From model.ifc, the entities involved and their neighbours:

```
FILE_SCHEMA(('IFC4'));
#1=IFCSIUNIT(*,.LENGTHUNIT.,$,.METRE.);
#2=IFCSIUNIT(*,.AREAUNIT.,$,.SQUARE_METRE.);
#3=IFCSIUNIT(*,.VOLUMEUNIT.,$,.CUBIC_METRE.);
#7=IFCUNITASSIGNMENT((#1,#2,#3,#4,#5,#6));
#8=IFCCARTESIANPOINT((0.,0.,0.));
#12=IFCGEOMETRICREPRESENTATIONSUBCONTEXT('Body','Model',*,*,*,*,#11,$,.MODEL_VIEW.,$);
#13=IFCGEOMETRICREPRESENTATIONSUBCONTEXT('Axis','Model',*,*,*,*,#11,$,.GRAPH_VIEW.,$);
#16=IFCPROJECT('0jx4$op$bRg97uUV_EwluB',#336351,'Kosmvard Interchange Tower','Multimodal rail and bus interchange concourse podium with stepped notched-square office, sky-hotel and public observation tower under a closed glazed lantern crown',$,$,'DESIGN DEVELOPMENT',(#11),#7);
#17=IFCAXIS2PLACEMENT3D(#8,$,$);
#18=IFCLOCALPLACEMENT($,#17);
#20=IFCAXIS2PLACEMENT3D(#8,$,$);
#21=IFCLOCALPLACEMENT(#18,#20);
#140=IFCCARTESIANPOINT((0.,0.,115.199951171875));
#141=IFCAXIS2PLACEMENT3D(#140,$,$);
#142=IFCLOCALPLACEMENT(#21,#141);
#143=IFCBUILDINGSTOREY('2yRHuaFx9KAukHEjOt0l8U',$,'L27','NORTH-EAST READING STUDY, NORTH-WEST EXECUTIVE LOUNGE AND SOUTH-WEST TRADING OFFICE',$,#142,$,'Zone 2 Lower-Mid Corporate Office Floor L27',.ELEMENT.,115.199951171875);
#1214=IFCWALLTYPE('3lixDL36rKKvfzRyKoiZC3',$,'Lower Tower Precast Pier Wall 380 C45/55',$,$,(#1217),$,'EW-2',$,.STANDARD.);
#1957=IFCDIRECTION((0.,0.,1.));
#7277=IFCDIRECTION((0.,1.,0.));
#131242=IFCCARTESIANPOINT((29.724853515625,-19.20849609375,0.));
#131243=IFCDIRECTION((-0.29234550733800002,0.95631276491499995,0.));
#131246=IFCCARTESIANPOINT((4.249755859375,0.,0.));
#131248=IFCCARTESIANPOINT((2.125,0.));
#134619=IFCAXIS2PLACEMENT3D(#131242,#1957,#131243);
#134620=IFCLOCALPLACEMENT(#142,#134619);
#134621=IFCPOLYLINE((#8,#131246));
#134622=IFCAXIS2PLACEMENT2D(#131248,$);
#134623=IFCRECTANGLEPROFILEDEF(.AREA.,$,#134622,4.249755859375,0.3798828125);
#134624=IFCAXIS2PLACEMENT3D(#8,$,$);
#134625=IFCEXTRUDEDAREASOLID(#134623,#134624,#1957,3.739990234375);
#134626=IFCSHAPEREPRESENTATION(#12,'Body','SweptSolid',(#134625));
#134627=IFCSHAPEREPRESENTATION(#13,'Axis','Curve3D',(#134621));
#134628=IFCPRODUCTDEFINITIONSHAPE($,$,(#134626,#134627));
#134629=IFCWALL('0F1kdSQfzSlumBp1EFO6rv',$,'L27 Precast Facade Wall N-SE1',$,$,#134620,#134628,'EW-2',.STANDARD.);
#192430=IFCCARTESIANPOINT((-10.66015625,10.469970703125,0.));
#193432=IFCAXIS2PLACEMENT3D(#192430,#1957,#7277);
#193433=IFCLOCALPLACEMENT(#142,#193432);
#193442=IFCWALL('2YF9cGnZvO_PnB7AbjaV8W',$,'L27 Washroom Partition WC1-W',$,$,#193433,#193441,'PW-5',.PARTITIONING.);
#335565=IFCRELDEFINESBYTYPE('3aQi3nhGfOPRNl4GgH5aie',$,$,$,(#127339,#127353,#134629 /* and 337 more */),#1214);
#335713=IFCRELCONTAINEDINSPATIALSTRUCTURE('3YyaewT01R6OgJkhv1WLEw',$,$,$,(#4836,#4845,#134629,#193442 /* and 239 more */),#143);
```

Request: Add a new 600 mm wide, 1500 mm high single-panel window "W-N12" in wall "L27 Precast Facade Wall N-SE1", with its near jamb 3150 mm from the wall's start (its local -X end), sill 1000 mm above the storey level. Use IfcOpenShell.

```python
import numpy as np
import ifcopenshell
import ifcopenshell.api.feature
import ifcopenshell.api.geometry
import ifcopenshell.api.root
import ifcopenshell.api.spatial
import ifcopenshell.geom
import ifcopenshell.util.element
import ifcopenshell.util.placement
import ifcopenshell.util.representation
import ifcopenshell.util.shape
import ifcopenshell.util.unit

model = ifcopenshell.open("model.ifc")
unit_scale = ifcopenshell.util.unit.calculate_unit_scale(model)
settings = ifcopenshell.geom.settings()


def volume(element):
    """Net volume in cubic metres, openings subtracted."""
    shape = ifcopenshell.geom.create_shape(settings, element)
    return ifcopenshell.util.shape.get_volume(shape.geometry)


wall = model.by_guid("0F1kdSQfzSlumBp1EFO6rv")
storey = ifcopenshell.util.element.get_container(wall, ifc_class="IfcBuildingStorey")
context = ifcopenshell.util.representation.get_context(model, "Model", "Body", "MODEL_VIEW")
before = volume(wall)

width, height, from_end, sill = 0.6, 1.5, 3.15, 1  # metres

# The wall runs along its own X axis, and the end named is its -X end.
wall_shape = ifcopenshell.geom.create_shape(settings, wall)
x, y, z = ifcopenshell.util.shape.get_vertices(wall_shape.geometry).T
start = x.min() + from_end
face, thickness = float(y.min()), float(y.max() - y.min())
wall_matrix = ifcopenshell.util.placement.get_local_placement(wall.ObjectPlacement)
level = ifcopenshell.util.placement.get_local_placement(storey.ObjectPlacement)[2, 3]


def in_wall(x, y):
    """Placement at x, y metres in the wall's axes, at sill height."""
    matrix = wall_matrix.copy()
    matrix[:, 3] = wall_matrix @ np.array([x / unit_scale, y / unit_scale, 0.0, 1.0])
    matrix[2, 3] = level + sill / unit_scale
    return matrix


# Opening: a box that overshoots both wall faces by 50 mm.
opening = ifcopenshell.api.root.create_entity(model, ifc_class="IfcOpeningElement", predefined_type="OPENING")
box = ifcopenshell.api.geometry.add_wall_representation(
    model, context=context, length=width, height=height, thickness=thickness + 0.1
)
ifcopenshell.api.geometry.assign_representation(model, product=opening, representation=box)
ifcopenshell.api.geometry.edit_object_placement(model, product=opening, matrix=in_wall(start, face - 0.05), is_si=False)
ifcopenshell.api.feature.add_feature(model, feature=opening, element=wall)

window = ifcopenshell.api.root.create_entity(model, ifc_class="IfcWindow", name="W-N12", predefined_type="WINDOW")
window.OverallWidth, window.OverallHeight = width / unit_scale, height / unit_scale
window.PartitioningType = "SINGLE_PANEL"
body = ifcopenshell.api.geometry.add_window_representation(
    model,
    context=context,
    overall_width=window.OverallWidth,
    overall_height=window.OverallHeight,
    partition_type="SINGLE_PANEL",
)
ifcopenshell.api.geometry.assign_representation(model, product=window, representation=body)
ifcopenshell.api.spatial.assign_container(model, products=[window], relating_structure=storey)
ifcopenshell.api.feature.add_filling(model, opening=opening, element=window)

# Centre the window in the wall's thickness.
ifcopenshell.api.geometry.edit_object_placement(model, product=window, matrix=in_wall(start, face), is_si=False)
window_shape = ifcopenshell.geom.create_shape(settings, window)
depth = ifcopenshell.util.shape.get_vertices(window_shape.geometry)[:, 1]
offset = face + thickness / 2 - (depth.min() + depth.max()) / 2
ifcopenshell.api.geometry.edit_object_placement(model, product=window, matrix=in_wall(start, offset), is_si=False)

after = volume(wall)

print(f"wall volume {before:.3f} -> {after:.3f} m3")

model.write("model_v2.ifc")
```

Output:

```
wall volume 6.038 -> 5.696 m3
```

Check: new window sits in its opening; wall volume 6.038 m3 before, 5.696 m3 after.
